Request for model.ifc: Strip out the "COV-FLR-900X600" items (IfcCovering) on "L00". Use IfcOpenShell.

First a look at what the model holds.

```python
import ifcopenshell
import ifcopenshell.util.element

model = ifcopenshell.open("model.ifc")
print(model.schema)
storey = next(s for s in model.by_type("IfcBuildingStorey") if s.Name == "L00")
coverings = [e for e in ifcopenshell.util.element.get_decomposition(storey) if e.is_a("IfcCovering")]
seen = {}
for e in coverings:
    element_type = ifcopenshell.util.element.get_type(e)
    name = element_type.Name if element_type not in (None, e) else None
    seen[name] = seen.get(name, 0) + 1
for name, count in sorted(seen.items(), key=str):
    print(count, "x", name)
```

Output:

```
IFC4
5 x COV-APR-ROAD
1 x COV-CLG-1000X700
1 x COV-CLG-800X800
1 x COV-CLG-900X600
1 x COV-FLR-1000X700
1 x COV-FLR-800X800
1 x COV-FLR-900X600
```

```python
import ifcopenshell
import ifcopenshell.api.root
import ifcopenshell.util.element

model = ifcopenshell.open("model.ifc")

storey = next(s for s in model.by_type("IfcBuildingStorey") if s.Name == "L00")
coverings = [e for e in ifcopenshell.util.element.get_decomposition(storey) if e.is_a("IfcCovering")]
targets = [e for e in coverings if (t := ifcopenshell.util.element.get_type(e)) not in (None, e) and t.Name == "COV-FLR-900X600"]

for e in targets:
    ifcopenshell.api.root.remove_product(model, product=e)
print(len(targets), "removed")

model.write("model_edited.ifc")
```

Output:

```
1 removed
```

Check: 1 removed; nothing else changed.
